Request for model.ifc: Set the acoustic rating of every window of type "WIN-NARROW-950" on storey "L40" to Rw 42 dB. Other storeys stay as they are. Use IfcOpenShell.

First a look at what the model holds.

```python
import ifcopenshell
import ifcopenshell.util.element

model = ifcopenshell.open("model.ifc")
print(model.schema)
storey = next(s for s in model.by_type("IfcBuildingStorey") if s.Name == "L40")
windows = [e for e in ifcopenshell.util.element.get_decomposition(storey) if e.is_a("IfcWindow")]
seen = {}
for e in windows:
    element_type = ifcopenshell.util.element.get_type(e)
    key = (element_type.Name if element_type != e and element_type else None, ifcopenshell.util.element.get_pset(e, "Pset_WindowCommon", "AcousticRating"))
    seen[key] = seen.get(key, 0) + 1
for (name, value), count in sorted(seen.items(), key=str):
    print(count, "x", name, "|", value)
```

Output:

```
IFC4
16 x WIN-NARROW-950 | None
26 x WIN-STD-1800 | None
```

```python
import ifcopenshell
import ifcopenshell.api.pset
import ifcopenshell.util.element

model = ifcopenshell.open("model.ifc")

storey = next(s for s in model.by_type("IfcBuildingStorey") if s.Name == "L40")
windows = [e for e in ifcopenshell.util.element.get_decomposition(storey) if e.is_a("IfcWindow")]

count = 0
for e in windows:
    element_type = ifcopenshell.util.element.get_type(e)
    if element_type in (None, e) or element_type.Name != "WIN-NARROW-950":
        continue
    found = ifcopenshell.util.element.get_pset(e, "Pset_WindowCommon", should_inherit=False)
    if found:
        pset = model.by_id(found["id"])
        if len(ifcopenshell.util.element.get_elements_by_pset(pset)) > 1:
            pset = ifcopenshell.api.pset.unshare_pset(model, products=[e], pset=pset)[0]
    else:
        pset = ifcopenshell.api.pset.add_pset(model, product=e, name="Pset_WindowCommon")
    ifcopenshell.api.pset.edit_pset(model, pset=pset, properties={"AcousticRating": "Rw 42 dB"})
    count += 1

print(count, "windows updated")

model.write("model-out.ifc")
```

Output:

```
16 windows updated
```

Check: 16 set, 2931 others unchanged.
